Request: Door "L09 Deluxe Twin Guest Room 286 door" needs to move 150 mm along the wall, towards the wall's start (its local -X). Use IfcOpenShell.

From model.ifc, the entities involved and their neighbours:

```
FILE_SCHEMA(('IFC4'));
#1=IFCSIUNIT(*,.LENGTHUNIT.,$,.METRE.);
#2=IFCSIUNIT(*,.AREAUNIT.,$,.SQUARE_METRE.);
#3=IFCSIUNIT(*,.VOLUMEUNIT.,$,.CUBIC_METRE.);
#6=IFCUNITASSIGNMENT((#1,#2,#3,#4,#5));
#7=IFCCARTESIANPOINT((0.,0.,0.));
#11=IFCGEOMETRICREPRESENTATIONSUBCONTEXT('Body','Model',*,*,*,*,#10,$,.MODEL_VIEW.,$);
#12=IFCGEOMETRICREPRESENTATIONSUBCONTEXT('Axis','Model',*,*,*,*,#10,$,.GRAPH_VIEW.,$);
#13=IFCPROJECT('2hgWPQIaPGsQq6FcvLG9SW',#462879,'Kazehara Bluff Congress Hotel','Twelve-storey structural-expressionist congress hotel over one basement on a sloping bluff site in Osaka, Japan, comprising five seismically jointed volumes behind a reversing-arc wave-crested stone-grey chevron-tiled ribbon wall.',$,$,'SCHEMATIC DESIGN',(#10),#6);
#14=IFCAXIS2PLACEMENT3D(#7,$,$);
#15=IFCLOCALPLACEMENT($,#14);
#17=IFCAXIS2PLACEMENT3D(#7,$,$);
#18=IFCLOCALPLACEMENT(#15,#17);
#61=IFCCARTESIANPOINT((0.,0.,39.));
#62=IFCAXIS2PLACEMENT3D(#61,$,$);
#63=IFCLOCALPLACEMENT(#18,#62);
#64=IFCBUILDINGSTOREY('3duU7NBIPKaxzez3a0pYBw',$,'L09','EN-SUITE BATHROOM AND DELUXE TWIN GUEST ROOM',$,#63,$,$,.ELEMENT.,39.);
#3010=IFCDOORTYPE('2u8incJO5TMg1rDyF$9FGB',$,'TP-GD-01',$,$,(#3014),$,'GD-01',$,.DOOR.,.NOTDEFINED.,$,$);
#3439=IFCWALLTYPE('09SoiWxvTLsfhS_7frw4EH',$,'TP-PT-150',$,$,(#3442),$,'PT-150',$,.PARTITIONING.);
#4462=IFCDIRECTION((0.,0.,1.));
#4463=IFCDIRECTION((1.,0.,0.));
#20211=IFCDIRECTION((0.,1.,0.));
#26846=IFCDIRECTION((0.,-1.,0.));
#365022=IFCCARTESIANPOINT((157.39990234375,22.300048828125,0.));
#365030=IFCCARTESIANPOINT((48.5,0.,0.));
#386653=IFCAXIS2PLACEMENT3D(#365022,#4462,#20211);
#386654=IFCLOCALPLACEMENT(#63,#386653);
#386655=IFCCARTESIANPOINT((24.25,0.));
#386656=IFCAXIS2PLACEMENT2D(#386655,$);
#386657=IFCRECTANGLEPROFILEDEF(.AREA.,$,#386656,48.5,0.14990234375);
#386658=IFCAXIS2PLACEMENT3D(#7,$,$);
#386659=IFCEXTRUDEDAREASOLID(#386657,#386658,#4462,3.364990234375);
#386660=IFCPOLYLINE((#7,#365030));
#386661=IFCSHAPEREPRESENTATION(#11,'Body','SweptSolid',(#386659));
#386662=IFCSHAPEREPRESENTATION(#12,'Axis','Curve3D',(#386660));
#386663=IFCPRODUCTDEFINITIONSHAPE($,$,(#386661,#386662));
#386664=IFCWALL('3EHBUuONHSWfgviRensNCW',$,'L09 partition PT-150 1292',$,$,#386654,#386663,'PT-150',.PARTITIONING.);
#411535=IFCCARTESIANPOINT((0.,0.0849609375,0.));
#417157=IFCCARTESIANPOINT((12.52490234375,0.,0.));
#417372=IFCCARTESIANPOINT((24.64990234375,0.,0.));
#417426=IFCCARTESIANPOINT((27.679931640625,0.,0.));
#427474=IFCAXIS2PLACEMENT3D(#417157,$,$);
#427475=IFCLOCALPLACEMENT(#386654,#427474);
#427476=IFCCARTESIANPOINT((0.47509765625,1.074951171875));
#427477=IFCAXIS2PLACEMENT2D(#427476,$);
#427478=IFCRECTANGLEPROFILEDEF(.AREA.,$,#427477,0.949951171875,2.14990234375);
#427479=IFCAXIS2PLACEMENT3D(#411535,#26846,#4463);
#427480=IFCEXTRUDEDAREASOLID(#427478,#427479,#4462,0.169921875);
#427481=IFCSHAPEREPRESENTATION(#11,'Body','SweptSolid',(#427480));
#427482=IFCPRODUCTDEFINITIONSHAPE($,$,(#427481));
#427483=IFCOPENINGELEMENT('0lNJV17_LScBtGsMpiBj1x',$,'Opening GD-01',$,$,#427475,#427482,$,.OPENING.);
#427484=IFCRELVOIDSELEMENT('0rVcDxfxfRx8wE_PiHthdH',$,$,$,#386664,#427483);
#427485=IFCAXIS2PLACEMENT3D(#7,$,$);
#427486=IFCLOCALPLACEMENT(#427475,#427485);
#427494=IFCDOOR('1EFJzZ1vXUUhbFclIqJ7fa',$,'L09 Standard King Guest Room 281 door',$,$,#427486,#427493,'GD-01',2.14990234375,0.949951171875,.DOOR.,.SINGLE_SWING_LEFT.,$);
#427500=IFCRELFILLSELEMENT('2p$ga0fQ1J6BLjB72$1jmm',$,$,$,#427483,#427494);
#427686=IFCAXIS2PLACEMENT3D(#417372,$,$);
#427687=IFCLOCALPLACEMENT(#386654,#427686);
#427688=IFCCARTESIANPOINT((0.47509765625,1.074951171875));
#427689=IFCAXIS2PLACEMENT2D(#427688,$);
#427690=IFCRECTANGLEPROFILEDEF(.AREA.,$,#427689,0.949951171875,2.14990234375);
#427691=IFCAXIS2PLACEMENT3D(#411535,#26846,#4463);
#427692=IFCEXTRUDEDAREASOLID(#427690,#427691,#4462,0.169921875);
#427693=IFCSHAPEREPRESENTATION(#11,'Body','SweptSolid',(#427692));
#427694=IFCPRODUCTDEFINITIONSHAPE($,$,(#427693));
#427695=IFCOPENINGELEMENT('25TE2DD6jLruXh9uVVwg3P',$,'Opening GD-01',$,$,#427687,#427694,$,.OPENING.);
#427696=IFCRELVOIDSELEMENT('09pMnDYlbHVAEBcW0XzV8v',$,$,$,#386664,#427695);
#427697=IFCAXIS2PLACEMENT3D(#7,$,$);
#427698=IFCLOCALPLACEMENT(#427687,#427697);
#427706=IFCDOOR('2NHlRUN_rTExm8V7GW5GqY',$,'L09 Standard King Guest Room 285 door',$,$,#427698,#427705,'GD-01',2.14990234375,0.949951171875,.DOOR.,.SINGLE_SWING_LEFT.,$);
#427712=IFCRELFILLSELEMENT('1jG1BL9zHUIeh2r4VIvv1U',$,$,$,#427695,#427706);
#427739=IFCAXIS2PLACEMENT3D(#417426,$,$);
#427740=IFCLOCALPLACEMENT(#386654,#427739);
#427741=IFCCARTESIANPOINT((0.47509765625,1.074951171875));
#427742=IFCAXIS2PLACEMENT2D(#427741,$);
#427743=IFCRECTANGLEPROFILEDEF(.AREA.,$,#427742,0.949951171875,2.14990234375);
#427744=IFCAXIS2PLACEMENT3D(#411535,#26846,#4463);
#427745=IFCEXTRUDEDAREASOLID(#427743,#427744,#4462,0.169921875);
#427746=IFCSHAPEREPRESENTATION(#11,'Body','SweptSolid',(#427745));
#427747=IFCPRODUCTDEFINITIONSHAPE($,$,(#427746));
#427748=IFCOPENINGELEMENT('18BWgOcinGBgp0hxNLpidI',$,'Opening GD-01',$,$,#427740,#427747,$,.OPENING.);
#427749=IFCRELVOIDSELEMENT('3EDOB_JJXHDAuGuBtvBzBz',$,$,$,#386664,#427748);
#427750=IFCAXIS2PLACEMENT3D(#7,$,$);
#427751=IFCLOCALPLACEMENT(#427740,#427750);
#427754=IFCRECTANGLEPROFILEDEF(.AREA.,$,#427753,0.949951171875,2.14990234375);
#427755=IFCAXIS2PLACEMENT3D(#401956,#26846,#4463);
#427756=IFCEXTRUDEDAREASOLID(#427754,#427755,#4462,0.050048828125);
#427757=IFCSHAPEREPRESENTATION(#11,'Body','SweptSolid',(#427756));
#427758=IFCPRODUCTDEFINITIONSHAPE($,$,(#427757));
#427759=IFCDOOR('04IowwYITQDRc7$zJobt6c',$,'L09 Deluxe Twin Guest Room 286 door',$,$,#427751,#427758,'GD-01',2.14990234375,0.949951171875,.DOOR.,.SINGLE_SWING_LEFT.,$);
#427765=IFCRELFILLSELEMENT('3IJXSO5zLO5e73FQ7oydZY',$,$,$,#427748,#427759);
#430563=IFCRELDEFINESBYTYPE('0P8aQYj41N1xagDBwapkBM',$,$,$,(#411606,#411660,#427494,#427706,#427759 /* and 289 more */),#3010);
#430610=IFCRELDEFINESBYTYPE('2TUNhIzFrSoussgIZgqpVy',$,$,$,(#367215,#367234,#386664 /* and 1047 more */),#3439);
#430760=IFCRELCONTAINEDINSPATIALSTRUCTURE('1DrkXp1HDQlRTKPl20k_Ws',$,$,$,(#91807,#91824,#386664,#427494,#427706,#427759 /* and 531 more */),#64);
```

```python
import ifcopenshell
import ifcopenshell.api.geometry
import ifcopenshell.util.placement
import ifcopenshell.util.unit

model = ifcopenshell.open("model.ifc")
unit_scale = ifcopenshell.util.unit.calculate_unit_scale(model)

door = model.by_id(427759)
opening = door.FillsVoids[0].RelatingOpeningElement
wall = opening.VoidsElements[0].RelatingBuildingElement

wall_matrix = ifcopenshell.util.placement.get_local_placement(wall.ObjectPlacement)
shift = wall_matrix[:3, 0] * -0.15 / unit_scale
before = ifcopenshell.util.placement.get_local_placement(door.ObjectPlacement)[:3, 3].copy()

# The door is placed relative to its opening, so it follows when the opening moves.
matrix = ifcopenshell.util.placement.get_local_placement(opening.ObjectPlacement)
matrix[:3, 3] += shift
ifcopenshell.api.geometry.edit_object_placement(
    model, product=opening, matrix=matrix, is_si=False, should_transform_children=True
)

after = ifcopenshell.util.placement.get_local_placement(door.ObjectPlacement)[:3, 3]
print("door moved by", (after - before).round(3) + 0.0)

model.write("model_updated.ifc")
```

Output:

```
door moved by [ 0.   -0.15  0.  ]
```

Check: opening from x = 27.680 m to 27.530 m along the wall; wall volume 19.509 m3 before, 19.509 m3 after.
